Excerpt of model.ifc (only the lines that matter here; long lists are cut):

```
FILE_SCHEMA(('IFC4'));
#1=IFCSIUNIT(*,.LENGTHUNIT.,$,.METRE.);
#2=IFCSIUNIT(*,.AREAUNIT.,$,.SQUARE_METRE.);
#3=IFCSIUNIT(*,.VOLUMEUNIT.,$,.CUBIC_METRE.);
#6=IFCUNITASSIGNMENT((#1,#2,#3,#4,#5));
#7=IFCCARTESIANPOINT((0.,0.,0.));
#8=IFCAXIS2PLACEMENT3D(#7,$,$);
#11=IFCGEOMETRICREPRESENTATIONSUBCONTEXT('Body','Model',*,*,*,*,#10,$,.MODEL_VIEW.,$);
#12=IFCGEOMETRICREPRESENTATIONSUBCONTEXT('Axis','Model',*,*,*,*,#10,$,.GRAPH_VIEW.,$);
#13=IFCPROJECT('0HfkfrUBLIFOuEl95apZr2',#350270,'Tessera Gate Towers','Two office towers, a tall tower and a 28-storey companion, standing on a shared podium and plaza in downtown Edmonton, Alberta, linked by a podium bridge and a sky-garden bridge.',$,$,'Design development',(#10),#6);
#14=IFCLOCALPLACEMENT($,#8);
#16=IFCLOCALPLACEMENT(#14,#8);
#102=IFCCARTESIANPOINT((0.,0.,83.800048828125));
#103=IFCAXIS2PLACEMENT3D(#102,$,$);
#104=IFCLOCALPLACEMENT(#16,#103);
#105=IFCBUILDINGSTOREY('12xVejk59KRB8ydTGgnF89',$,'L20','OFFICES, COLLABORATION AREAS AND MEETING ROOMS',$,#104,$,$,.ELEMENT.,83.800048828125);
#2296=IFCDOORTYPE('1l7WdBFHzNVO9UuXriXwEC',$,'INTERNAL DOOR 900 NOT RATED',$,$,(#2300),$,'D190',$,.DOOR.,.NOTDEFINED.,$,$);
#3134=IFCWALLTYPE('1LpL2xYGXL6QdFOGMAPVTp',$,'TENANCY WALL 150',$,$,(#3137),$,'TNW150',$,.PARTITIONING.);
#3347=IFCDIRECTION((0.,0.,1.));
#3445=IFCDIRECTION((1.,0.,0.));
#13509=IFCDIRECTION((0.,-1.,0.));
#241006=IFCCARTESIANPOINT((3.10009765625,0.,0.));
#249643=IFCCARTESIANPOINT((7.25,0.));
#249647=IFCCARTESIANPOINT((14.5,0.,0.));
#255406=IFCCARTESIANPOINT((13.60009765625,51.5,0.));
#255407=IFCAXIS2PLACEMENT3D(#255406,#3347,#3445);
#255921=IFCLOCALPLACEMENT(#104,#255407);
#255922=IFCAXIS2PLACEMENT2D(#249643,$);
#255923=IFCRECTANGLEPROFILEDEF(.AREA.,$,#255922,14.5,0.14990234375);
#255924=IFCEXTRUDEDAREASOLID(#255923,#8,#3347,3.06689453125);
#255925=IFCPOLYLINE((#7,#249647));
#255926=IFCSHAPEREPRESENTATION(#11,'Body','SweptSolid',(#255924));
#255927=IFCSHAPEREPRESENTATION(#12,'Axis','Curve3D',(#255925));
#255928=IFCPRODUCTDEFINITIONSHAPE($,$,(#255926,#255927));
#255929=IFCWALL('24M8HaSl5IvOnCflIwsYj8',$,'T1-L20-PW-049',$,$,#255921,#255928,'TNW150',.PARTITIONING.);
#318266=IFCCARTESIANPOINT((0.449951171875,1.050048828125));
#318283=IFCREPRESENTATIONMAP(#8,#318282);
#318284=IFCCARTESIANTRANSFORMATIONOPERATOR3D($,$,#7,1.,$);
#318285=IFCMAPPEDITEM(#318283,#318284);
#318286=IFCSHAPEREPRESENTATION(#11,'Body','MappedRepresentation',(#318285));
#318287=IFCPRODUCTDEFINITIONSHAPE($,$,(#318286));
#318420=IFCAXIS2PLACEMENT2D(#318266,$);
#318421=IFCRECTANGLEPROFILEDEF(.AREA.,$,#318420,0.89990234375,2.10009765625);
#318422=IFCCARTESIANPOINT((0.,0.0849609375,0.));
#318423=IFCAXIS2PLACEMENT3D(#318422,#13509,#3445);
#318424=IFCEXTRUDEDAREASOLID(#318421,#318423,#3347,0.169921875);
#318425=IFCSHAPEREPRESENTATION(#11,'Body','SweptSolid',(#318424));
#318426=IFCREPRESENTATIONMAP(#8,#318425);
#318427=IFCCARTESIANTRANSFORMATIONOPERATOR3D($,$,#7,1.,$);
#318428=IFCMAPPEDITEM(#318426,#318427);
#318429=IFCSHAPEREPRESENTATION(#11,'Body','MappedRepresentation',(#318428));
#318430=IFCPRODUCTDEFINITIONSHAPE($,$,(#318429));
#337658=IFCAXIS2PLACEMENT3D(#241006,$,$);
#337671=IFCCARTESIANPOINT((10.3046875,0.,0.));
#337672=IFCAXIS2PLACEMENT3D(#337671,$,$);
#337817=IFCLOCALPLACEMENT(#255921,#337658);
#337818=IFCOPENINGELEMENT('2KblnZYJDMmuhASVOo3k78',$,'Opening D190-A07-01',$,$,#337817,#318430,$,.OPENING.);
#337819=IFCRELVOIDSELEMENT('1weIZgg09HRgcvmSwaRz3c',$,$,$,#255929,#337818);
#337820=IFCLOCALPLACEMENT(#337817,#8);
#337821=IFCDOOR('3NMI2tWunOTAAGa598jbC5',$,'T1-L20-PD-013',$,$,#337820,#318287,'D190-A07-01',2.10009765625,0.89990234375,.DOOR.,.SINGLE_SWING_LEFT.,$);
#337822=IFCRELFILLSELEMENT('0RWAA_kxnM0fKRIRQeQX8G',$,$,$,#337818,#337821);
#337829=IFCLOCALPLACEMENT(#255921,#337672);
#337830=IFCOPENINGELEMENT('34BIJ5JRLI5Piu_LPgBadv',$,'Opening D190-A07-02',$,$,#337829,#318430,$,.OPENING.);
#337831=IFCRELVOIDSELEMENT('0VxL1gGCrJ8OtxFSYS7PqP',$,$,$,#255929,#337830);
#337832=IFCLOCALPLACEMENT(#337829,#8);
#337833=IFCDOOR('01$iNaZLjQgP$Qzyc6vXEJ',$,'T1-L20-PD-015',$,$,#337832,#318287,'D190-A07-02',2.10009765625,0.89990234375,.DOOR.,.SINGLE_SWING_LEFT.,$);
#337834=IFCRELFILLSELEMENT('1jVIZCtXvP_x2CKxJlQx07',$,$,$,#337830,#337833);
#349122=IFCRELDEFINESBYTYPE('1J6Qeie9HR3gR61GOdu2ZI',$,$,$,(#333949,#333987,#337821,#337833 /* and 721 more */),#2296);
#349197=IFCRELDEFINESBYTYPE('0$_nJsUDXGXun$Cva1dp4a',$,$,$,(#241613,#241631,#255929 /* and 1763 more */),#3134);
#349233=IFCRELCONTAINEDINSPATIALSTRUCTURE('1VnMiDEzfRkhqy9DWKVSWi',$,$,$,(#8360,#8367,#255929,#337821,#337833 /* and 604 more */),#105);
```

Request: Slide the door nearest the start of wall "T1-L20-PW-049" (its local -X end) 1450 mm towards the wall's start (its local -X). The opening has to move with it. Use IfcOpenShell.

```python
import ifcopenshell
import ifcopenshell.api.geometry
import ifcopenshell.util.placement

model = ifcopenshell.open("model.ifc")

door = model.by_guid("3NMI2tWunOTAAGa598jbC5")
opening = door.FillsVoids[0].RelatingOpeningElement
wall = opening.VoidsElements[0].RelatingBuildingElement

wall_matrix = ifcopenshell.util.placement.get_local_placement(wall.ObjectPlacement)
shift = wall_matrix[:3, 0] * -1.45
before = ifcopenshell.util.placement.get_local_placement(door.ObjectPlacement)[:3, 3].copy()

# The door is placed relative to its opening, so it follows when the opening moves.
matrix = ifcopenshell.util.placement.get_local_placement(opening.ObjectPlacement)
matrix[:3, 3] += shift
ifcopenshell.api.geometry.edit_object_placement(
    model, product=opening, matrix=matrix, is_si=False, should_transform_children=True
)

after = ifcopenshell.util.placement.get_local_placement(door.ObjectPlacement)[:3, 3]
print("door moved by", (after - before).round(3) + 0.0)

model.write("model_updated.ifc")
```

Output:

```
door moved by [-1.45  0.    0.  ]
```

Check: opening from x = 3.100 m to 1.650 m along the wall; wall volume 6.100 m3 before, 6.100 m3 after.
